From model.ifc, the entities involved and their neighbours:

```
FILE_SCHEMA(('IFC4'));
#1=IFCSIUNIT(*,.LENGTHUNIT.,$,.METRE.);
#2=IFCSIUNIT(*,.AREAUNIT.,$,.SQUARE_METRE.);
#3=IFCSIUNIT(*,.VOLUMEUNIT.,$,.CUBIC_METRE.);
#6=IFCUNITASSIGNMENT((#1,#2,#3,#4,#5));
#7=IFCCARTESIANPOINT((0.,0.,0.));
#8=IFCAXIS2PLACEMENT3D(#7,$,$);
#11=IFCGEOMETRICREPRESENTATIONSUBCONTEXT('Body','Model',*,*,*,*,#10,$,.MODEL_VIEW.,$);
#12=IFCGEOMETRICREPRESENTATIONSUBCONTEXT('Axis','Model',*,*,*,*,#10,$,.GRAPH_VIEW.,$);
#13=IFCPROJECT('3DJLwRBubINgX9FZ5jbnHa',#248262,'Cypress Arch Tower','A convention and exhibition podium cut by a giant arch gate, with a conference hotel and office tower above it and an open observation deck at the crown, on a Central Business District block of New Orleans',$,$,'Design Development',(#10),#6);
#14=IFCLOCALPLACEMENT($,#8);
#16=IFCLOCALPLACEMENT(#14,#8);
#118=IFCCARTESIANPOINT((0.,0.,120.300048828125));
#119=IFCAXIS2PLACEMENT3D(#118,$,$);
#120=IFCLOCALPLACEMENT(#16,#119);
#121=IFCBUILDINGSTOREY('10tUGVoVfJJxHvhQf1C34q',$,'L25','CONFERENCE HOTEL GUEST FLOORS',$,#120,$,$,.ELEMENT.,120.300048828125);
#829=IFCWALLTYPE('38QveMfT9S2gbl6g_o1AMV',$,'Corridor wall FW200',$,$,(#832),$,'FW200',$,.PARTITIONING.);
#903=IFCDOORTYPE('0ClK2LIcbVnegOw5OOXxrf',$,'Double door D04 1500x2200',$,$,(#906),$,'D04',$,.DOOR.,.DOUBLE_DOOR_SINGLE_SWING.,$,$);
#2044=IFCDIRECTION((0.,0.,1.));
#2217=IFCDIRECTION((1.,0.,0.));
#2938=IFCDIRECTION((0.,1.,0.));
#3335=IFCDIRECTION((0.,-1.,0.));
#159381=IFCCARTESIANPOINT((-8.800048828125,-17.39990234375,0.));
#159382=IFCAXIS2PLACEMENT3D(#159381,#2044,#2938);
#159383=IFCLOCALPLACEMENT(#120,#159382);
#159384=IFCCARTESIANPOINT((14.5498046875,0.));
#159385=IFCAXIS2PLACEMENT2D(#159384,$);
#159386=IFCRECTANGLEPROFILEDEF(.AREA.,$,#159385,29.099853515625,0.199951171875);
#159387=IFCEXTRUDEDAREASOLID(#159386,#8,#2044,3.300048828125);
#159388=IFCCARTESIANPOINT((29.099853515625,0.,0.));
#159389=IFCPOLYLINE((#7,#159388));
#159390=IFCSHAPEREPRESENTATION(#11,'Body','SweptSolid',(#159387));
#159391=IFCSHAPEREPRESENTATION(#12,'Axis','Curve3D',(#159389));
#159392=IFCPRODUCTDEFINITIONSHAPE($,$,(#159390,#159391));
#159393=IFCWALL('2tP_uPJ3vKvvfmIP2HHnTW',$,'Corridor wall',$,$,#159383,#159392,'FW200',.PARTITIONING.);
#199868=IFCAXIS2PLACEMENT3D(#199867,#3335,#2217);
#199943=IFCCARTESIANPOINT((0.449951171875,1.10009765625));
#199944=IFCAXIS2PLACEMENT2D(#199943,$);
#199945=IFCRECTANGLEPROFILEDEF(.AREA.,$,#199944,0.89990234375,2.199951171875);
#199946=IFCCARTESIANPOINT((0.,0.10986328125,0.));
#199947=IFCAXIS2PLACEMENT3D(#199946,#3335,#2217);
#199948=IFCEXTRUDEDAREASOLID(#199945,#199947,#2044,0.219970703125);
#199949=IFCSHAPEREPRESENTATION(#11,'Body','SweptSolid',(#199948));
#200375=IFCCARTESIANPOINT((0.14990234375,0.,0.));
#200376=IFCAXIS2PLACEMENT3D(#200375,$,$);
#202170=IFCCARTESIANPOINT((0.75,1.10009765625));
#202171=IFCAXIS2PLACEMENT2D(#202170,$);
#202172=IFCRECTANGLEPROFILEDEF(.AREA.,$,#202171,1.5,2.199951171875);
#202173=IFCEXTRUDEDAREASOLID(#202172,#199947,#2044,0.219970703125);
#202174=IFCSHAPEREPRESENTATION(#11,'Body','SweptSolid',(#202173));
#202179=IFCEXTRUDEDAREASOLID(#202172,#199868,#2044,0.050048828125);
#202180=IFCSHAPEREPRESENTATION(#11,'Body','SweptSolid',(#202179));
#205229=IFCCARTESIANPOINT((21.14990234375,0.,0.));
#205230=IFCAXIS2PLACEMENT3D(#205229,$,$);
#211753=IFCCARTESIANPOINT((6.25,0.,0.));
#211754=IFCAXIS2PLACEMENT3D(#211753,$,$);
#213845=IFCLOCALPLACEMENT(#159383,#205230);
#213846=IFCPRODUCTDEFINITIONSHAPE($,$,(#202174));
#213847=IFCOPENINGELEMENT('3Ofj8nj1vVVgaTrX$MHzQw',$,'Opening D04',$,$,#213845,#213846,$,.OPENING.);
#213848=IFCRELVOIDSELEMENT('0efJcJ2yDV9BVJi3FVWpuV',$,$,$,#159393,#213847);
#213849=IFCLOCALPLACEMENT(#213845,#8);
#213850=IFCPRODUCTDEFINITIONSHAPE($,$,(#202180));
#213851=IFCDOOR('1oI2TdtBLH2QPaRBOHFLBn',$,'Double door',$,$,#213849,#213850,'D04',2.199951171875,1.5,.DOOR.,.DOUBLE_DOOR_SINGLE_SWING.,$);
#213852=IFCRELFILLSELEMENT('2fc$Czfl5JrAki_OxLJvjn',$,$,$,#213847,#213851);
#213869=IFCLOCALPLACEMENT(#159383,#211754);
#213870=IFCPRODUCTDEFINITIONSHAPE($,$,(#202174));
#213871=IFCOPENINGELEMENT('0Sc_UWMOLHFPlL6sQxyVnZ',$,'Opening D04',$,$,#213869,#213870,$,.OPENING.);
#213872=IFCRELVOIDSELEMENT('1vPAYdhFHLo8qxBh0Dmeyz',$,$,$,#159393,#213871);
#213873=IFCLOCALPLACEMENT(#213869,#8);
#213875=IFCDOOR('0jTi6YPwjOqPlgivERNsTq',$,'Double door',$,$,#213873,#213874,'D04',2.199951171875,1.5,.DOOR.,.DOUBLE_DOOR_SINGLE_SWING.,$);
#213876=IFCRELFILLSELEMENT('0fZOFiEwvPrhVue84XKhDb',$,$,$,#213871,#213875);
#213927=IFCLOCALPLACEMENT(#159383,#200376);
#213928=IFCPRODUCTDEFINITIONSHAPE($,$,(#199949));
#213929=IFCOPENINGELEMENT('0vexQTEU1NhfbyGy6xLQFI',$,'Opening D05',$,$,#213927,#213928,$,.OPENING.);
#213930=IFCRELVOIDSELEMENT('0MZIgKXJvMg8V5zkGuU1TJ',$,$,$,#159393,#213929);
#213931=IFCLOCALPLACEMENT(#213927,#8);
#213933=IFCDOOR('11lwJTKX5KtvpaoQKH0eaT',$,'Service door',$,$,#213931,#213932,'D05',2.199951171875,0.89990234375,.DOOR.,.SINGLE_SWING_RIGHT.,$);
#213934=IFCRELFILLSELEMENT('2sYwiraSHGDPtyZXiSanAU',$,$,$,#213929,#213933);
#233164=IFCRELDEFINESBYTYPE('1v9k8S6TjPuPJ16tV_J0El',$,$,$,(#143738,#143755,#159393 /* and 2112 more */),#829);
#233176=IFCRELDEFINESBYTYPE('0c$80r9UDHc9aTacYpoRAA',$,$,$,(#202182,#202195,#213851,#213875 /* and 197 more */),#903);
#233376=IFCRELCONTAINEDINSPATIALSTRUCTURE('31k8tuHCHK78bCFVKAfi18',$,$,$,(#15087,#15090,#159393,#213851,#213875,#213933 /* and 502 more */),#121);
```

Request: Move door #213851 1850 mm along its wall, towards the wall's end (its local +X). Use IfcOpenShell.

```python
import ifcopenshell
import ifcopenshell.api.geometry
import ifcopenshell.util.placement
import ifcopenshell.util.unit

model = ifcopenshell.open("model.ifc")
unit_scale = ifcopenshell.util.unit.calculate_unit_scale(model)

door = model.by_guid("1oI2TdtBLH2QPaRBOHFLBn")
opening = door.FillsVoids[0].RelatingOpeningElement
wall = opening.VoidsElements[0].RelatingBuildingElement

wall_matrix = ifcopenshell.util.placement.get_local_placement(wall.ObjectPlacement)
shift = wall_matrix[:3, 0] * 1.85 / unit_scale
before = ifcopenshell.util.placement.get_local_placement(door.ObjectPlacement)[:3, 3].copy()

# The door is placed relative to its opening, so it follows when the opening moves.
matrix = ifcopenshell.util.placement.get_local_placement(opening.ObjectPlacement)
matrix[:3, 3] += shift
ifcopenshell.api.geometry.edit_object_placement(
    model, product=opening, matrix=matrix, is_si=False, should_transform_children=True
)

after = ifcopenshell.util.placement.get_local_placement(door.ObjectPlacement)[:3, 3]
print("door moved by", (after - before).round(3) + 0.0)

model.write("model-out.ifc")
```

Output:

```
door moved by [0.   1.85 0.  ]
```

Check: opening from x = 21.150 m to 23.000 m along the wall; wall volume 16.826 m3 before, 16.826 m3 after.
